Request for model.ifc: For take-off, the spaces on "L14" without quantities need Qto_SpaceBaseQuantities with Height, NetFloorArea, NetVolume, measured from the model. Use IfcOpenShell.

First a look at what the model holds.

```python
import ifcopenshell
import ifcopenshell.util.element
import ifcopenshell.util.unit

model = ifcopenshell.open("model.ifc")
print(model.schema)
for unit_type in ("LENGTHUNIT", "AREAUNIT", "VOLUMEUNIT"):
    print(unit_type, ifcopenshell.util.unit.calculate_unit_scale(model, unit_type))
storey = next(s for s in model.by_type("IfcBuildingStorey") if s.Name == "L14")
spaces = [e for e in ifcopenshell.util.element.get_decomposition(storey) if e.is_a("IfcSpace")]
for e in sorted(spaces, key=lambda e: e.id()):
    print(e.id(), e.is_a(), e.Name, list(ifcopenshell.util.element.get_psets(e, qtos_only=True)), sep=" | ")
```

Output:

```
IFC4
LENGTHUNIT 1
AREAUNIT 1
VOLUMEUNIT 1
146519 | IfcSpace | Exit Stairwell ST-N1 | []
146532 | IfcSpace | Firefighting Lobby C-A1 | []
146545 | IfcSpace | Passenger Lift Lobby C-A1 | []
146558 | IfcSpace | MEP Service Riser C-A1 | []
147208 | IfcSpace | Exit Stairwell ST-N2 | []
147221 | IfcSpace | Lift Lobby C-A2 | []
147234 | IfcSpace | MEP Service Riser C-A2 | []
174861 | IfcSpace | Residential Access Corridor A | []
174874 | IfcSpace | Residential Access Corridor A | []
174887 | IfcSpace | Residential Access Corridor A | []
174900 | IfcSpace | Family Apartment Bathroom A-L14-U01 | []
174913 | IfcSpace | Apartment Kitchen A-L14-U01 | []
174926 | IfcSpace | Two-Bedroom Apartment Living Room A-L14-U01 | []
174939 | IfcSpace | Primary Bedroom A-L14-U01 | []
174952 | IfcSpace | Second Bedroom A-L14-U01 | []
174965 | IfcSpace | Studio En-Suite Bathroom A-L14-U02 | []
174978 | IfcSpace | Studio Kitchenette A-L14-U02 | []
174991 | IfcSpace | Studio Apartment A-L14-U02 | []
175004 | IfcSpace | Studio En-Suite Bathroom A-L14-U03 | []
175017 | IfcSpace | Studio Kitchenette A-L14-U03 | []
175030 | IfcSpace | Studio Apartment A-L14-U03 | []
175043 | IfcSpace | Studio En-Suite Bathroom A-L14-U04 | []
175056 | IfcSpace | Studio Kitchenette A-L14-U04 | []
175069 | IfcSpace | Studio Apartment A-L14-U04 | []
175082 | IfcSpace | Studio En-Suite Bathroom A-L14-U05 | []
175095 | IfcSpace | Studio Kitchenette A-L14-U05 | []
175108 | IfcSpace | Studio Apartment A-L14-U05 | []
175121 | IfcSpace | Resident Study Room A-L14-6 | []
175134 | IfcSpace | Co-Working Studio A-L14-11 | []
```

```python
import ifcopenshell
import ifcopenshell.api.pset
import ifcopenshell.geom
import ifcopenshell.util.element
import ifcopenshell.util.shape
import ifcopenshell.util.unit

model = ifcopenshell.open("model.ifc")
unit_scale = ifcopenshell.util.unit.calculate_unit_scale(model)
area_scale = ifcopenshell.util.unit.calculate_unit_scale(model, "AREAUNIT")
volume_scale = ifcopenshell.util.unit.calculate_unit_scale(model, "VOLUMEUNIT")
settings = ifcopenshell.geom.settings()

storey = next(s for s in model.by_type("IfcBuildingStorey") if s.Name == "L14")
spaces = [e for e in ifcopenshell.util.element.get_decomposition(storey) if e.is_a("IfcSpace")]

for e in sorted(spaces, key=lambda e: e.id()):
    if ifcopenshell.util.element.get_psets(e, qtos_only=True, should_inherit=False):
        continue
    # Geometry comes back in metres, in the element's own axes.
    shape = ifcopenshell.geom.create_shape(settings, e)
    values = {
        "Height": ifcopenshell.util.shape.get_z(shape.geometry) / unit_scale,
        "NetFloorArea": ifcopenshell.util.shape.get_footprint_area(shape.geometry) / area_scale,
        "NetVolume": ifcopenshell.util.shape.get_volume(shape.geometry) / volume_scale,
    }
    qto = ifcopenshell.api.pset.add_qto(model, product=e, name="Qto_SpaceBaseQuantities")
    ifcopenshell.api.pset.edit_qto(model, qto=qto, properties=values)
    print(e.id(), {k: round(v, 3) for k, v in values.items()})

model.write("model-out.ifc")
```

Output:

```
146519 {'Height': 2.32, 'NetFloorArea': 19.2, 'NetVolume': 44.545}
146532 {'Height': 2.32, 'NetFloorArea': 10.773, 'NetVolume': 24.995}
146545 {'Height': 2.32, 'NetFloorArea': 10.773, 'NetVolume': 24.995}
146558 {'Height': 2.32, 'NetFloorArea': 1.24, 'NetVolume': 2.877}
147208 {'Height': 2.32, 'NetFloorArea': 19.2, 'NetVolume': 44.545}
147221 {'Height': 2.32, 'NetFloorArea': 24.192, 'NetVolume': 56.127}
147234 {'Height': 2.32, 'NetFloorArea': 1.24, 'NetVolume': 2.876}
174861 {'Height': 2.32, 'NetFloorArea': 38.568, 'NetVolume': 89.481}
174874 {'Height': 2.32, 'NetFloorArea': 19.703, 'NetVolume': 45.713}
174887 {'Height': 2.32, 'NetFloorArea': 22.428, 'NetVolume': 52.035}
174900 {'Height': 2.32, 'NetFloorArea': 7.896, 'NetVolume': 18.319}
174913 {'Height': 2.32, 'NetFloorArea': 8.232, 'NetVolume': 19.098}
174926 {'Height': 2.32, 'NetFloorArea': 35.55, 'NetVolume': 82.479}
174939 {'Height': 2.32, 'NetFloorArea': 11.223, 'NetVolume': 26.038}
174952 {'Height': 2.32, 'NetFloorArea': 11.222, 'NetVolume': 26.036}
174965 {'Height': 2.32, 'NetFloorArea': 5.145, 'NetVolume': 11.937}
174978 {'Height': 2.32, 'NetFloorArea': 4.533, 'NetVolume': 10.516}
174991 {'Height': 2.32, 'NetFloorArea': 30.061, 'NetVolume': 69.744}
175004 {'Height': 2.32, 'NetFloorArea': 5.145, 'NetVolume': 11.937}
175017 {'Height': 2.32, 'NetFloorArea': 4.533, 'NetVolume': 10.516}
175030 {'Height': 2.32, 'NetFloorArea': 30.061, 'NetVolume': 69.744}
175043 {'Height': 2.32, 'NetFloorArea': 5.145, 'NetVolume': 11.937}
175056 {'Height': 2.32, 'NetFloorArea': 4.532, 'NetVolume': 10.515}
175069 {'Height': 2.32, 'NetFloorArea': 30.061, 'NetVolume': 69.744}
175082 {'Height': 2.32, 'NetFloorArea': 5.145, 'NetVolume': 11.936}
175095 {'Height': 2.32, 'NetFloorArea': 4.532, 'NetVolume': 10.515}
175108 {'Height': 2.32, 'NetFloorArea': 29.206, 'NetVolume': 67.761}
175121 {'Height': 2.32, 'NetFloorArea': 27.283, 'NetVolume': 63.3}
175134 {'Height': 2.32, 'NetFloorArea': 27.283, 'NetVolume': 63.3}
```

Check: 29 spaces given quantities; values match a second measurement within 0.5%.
